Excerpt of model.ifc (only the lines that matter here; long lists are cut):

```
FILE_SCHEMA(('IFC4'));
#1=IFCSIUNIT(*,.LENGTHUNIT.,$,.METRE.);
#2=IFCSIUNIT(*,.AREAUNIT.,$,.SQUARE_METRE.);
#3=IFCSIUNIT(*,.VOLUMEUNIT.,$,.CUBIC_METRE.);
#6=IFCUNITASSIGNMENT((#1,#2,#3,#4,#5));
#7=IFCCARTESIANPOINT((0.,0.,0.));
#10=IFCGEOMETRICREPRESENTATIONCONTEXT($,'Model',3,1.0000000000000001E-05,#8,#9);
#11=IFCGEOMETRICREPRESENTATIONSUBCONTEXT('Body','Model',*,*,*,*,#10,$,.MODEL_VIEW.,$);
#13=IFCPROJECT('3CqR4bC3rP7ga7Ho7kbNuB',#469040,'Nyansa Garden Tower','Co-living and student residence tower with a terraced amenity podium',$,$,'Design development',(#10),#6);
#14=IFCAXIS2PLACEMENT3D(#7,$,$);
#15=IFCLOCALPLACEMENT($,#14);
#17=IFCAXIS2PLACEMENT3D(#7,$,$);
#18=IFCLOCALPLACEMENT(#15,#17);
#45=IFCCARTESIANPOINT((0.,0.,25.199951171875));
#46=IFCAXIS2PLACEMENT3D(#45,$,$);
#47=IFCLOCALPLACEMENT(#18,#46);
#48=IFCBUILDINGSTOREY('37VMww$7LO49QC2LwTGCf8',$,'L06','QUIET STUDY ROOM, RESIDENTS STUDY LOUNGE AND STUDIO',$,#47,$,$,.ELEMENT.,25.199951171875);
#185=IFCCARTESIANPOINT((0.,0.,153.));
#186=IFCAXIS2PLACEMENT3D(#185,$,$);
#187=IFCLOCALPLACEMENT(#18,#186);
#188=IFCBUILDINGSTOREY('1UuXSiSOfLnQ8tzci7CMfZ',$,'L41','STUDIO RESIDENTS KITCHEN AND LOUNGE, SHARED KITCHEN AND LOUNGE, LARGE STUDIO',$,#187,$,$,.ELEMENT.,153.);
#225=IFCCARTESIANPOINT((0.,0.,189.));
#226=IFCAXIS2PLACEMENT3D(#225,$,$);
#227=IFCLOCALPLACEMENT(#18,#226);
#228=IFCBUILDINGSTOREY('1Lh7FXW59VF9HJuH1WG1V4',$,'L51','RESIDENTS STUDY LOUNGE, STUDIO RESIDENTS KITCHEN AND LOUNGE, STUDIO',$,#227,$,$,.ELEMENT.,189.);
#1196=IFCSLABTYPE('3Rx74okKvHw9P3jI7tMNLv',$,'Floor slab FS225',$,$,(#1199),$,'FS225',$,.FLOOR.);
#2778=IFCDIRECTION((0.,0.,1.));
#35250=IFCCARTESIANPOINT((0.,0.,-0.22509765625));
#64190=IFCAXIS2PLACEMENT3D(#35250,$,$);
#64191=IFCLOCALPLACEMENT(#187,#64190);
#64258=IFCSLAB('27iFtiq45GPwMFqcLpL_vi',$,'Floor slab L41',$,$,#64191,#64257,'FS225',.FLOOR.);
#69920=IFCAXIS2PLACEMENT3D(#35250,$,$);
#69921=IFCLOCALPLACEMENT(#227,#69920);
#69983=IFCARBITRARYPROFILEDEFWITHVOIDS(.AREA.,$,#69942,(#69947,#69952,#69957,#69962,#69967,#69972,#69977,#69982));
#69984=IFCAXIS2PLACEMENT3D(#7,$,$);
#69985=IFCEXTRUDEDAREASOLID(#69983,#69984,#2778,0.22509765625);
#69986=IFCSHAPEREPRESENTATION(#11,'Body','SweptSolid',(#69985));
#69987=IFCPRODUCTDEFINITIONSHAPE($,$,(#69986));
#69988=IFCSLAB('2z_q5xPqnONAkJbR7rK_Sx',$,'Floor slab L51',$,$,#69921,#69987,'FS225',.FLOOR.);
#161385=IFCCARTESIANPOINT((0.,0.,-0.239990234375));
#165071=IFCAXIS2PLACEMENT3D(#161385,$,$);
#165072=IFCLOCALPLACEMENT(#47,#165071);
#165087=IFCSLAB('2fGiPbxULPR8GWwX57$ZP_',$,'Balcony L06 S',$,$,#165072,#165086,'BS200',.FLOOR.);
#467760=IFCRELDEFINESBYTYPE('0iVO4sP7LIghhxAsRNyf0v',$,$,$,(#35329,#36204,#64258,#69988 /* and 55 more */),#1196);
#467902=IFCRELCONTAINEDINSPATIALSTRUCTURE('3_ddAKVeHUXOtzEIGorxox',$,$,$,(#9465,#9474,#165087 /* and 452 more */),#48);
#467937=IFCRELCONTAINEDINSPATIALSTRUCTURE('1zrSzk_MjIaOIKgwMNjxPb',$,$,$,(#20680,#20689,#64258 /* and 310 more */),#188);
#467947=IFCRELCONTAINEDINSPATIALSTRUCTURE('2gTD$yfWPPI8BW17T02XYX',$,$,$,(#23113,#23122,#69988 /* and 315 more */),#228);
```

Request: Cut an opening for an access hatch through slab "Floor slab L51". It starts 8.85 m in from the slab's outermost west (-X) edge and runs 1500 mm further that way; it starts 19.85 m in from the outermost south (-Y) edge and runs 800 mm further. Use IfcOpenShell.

```python
import numpy as np
import ifcopenshell
import ifcopenshell.api.feature
import ifcopenshell.api.geometry
import ifcopenshell.api.root
import ifcopenshell.geom
import ifcopenshell.util.placement
import ifcopenshell.util.representation
import ifcopenshell.util.shape
import ifcopenshell.util.unit

model = ifcopenshell.open("model.ifc")
unit_scale = ifcopenshell.util.unit.calculate_unit_scale(model)
settings = ifcopenshell.geom.settings()


def volume(element):
    """Net volume in cubic metres, openings subtracted."""
    shape = ifcopenshell.geom.create_shape(settings, element)
    return ifcopenshell.util.shape.get_volume(shape.geometry)


slab = model.by_guid("2z_q5xPqnONAkJbR7rK_Sx")
before = volume(slab)

# Extent in the slab's own axes, in metres. The edges named are its -X and -Y sides.
slab_shape = ifcopenshell.geom.create_shape(settings, slab)
vertices = ifcopenshell.util.shape.get_vertices(slab_shape.geometry)
x_min, y_min, bottom = vertices.min(axis=0)
top = vertices[:, 2].max()

opening = ifcopenshell.api.root.create_entity(model, ifc_class="IfcOpeningElement", name="Access hatch opening", predefined_type="OPENING")
context = ifcopenshell.util.representation.get_context(model, "Model", "Body", "MODEL_VIEW")
width, depth = 1.5, 0.8
outline = [(0.0, 0.0), (width, 0.0), (width, depth), (0.0, depth), (0.0, 0.0)]
# Overshoot both faces by 50 mm so the cut is clean.
shape = ifcopenshell.api.geometry.add_slab_representation(
    model, context=context, depth=top - bottom + 0.1, polyline=outline
)
ifcopenshell.api.geometry.assign_representation(model, product=opening, representation=shape)

matrix = ifcopenshell.util.placement.get_local_placement(slab.ObjectPlacement)
matrix[:, 3] = matrix @ np.append(np.array([x_min + 8.85, y_min + 19.85, bottom - 0.05]) / unit_scale, 1.0)
ifcopenshell.api.geometry.edit_object_placement(model, product=opening, matrix=matrix, is_si=False)
ifcopenshell.api.feature.add_feature(model, feature=opening, element=slab)

after = volume(slab)

print(f"slab volume {before:.3f} -> {after:.3f} m3")

model.write("model_rev.ifc")
```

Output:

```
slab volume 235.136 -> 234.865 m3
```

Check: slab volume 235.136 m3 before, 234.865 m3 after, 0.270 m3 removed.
